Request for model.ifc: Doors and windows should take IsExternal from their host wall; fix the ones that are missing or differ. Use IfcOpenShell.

First a look at what the model holds.

```python
import ifcopenshell
import ifcopenshell.util.element

model = ifcopenshell.open("model.ifc")
print(model.schema)
seen = {}
for e in model.by_type("IfcDoor") + model.by_type("IfcWindow"):
    if not e.FillsVoids:
        continue
    host = e.FillsVoids[0].RelatingOpeningElement.VoidsElements[0].RelatingBuildingElement
    own = ifcopenshell.util.element.get_pset(e, f"Pset_{e.is_a()[3:].removesuffix('StandardCase')}Common", "IsExternal")
    wall = ifcopenshell.util.element.get_pset(host, "Pset_WallCommon", "IsExternal")
    seen[e.is_a(), own, wall] = seen.get((e.is_a(), own, wall), 0) + 1
for (cls, own, wall), count in sorted(seen.items(), key=str):
    print(count, cls, "IsExternal:", own, "| host wall:", wall)
```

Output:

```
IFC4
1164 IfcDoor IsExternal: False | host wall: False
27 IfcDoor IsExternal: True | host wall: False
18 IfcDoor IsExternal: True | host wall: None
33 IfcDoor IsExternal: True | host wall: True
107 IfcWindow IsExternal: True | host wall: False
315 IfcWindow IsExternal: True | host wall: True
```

```python
import ifcopenshell
import ifcopenshell.api.pset
import ifcopenshell.util.element

model = ifcopenshell.open("model.ifc")

count = 0
for ifc_class, pset_name in (("IfcDoor", "Pset_DoorCommon"), ("IfcWindow", "Pset_WindowCommon")):
    for e in model.by_type(ifc_class):
        if not e.FillsVoids:
            continue
        host = e.FillsVoids[0].RelatingOpeningElement.VoidsElements[0].RelatingBuildingElement
        external = ifcopenshell.util.element.get_pset(host, "Pset_WallCommon", "IsExternal")
        if external is None or ifcopenshell.util.element.get_pset(e, pset_name, "IsExternal") == external:
            continue
        pset = ifcopenshell.api.pset.add_pset(model, product=e, name=pset_name)
        ifcopenshell.api.pset.edit_pset(model, pset=pset, properties={"IsExternal": external})
        count += 1

print(count, "updated")

model.write("model_edited.ifc")
```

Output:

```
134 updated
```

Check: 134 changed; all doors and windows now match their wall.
